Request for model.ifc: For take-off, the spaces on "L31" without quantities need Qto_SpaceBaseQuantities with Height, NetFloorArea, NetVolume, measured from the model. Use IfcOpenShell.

First a look at what the model holds.

```python
import ifcopenshell
import ifcopenshell.util.element
import ifcopenshell.util.unit

model = ifcopenshell.open("model.ifc")
print(model.schema)
for unit_type in ("LENGTHUNIT", "AREAUNIT", "VOLUMEUNIT"):
    print(unit_type, ifcopenshell.util.unit.calculate_unit_scale(model, unit_type))
storey = next(s for s in model.by_type("IfcBuildingStorey") if s.Name == "L31")
spaces = [e for e in ifcopenshell.util.element.get_decomposition(storey) if e.is_a("IfcSpace")]
for e in sorted(spaces, key=lambda e: e.id()):
    print(e.id(), e.is_a(), e.Name, list(ifcopenshell.util.element.get_psets(e, qtos_only=True)), sep=" | ")
```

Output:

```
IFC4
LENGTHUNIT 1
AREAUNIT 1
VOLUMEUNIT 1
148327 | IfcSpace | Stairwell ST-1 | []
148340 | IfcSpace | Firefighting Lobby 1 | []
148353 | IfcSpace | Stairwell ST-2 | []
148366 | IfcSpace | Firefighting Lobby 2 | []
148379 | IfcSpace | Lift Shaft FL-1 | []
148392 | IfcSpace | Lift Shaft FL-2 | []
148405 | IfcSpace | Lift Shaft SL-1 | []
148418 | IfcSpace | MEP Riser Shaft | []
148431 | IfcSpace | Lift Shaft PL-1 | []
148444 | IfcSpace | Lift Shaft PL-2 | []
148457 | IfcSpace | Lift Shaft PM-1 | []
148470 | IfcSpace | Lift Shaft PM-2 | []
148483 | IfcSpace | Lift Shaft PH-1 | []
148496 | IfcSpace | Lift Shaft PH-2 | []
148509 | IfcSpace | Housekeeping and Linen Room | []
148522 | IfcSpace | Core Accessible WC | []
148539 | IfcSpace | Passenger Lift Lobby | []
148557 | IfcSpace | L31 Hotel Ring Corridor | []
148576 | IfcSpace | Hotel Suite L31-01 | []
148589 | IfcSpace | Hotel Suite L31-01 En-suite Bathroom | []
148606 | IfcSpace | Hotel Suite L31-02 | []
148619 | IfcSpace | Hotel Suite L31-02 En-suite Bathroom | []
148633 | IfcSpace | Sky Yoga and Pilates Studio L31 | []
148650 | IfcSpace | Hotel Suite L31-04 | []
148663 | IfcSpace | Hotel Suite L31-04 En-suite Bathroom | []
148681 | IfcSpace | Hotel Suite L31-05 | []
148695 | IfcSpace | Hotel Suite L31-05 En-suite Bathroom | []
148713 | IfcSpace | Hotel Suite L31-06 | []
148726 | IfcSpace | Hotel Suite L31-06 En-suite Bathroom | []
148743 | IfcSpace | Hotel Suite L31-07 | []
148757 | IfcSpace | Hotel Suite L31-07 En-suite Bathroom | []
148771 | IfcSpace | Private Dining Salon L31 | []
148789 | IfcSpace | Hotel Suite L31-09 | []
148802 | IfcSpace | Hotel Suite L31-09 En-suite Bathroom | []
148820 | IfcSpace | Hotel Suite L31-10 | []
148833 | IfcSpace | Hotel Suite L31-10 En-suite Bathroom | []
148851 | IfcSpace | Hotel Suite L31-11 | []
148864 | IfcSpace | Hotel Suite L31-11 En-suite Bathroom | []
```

```python
import ifcopenshell
import ifcopenshell.api.pset
import ifcopenshell.geom
import ifcopenshell.util.element
import ifcopenshell.util.shape
import ifcopenshell.util.unit

model = ifcopenshell.open("model.ifc")
unit_scale = ifcopenshell.util.unit.calculate_unit_scale(model)
area_scale = ifcopenshell.util.unit.calculate_unit_scale(model, "AREAUNIT")
volume_scale = ifcopenshell.util.unit.calculate_unit_scale(model, "VOLUMEUNIT")
settings = ifcopenshell.geom.settings()

storey = next(s for s in model.by_type("IfcBuildingStorey") if s.Name == "L31")
spaces = [e for e in ifcopenshell.util.element.get_decomposition(storey) if e.is_a("IfcSpace")]

for e in sorted(spaces, key=lambda e: e.id()):
    if ifcopenshell.util.element.get_psets(e, qtos_only=True, should_inherit=False):
        continue
    # Geometry comes back in metres, in the element's own axes.
    shape = ifcopenshell.geom.create_shape(settings, e)
    values = {
        "Height": ifcopenshell.util.shape.get_z(shape.geometry) / unit_scale,
        "NetFloorArea": ifcopenshell.util.shape.get_footprint_area(shape.geometry) / area_scale,
        "NetVolume": ifcopenshell.util.shape.get_volume(shape.geometry) / volume_scale,
    }
    qto = ifcopenshell.api.pset.add_qto(model, product=e, name="Qto_SpaceBaseQuantities")
    ifcopenshell.api.pset.edit_qto(model, qto=qto, properties=values)
    print(e.id(), {k: round(v, 3) for k, v in values.items()})

model.write("model_updated.ifc")
```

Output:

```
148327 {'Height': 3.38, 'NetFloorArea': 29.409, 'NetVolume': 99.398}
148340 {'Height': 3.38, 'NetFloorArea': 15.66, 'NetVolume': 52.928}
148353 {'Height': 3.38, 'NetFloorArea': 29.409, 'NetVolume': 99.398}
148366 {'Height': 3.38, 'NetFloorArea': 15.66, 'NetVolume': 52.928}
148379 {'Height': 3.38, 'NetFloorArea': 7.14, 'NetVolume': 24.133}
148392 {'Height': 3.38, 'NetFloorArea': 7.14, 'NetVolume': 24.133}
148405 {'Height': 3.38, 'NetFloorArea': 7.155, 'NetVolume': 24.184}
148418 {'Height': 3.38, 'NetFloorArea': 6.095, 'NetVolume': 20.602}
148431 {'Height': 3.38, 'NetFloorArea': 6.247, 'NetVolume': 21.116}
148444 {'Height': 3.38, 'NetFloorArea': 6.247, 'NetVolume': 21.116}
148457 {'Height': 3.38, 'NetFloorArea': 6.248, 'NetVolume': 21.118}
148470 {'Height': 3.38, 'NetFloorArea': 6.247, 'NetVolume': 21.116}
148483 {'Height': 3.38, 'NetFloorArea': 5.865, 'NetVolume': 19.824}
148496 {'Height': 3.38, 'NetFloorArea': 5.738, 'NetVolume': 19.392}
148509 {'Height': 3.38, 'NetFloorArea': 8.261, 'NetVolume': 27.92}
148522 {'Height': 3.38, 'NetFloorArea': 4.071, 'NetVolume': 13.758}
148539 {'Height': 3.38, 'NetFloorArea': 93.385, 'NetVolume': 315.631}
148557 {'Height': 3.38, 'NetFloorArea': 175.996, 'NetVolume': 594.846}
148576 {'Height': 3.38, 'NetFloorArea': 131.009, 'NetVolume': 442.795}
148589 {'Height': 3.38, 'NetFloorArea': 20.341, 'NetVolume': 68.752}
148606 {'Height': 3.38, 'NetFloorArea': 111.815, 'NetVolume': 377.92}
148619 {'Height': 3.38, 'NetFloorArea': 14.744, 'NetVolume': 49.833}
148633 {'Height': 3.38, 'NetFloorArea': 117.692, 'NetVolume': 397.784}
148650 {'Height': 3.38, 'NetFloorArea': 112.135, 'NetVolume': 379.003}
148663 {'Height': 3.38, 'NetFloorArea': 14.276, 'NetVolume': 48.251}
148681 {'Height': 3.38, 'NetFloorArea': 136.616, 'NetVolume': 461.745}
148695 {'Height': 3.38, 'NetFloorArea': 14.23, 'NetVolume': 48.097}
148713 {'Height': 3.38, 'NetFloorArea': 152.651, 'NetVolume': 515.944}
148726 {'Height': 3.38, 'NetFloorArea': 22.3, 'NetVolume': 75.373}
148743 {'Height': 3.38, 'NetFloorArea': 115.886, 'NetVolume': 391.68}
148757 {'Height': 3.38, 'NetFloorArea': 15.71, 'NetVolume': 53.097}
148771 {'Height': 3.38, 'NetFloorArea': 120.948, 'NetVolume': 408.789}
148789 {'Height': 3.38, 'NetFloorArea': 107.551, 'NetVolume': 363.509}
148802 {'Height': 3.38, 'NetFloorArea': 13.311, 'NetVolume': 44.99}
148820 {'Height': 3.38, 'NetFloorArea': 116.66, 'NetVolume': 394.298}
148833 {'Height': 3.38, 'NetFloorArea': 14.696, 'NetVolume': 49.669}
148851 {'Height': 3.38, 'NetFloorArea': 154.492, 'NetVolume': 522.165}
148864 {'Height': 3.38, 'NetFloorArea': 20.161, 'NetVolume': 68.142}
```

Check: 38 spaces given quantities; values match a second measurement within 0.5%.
